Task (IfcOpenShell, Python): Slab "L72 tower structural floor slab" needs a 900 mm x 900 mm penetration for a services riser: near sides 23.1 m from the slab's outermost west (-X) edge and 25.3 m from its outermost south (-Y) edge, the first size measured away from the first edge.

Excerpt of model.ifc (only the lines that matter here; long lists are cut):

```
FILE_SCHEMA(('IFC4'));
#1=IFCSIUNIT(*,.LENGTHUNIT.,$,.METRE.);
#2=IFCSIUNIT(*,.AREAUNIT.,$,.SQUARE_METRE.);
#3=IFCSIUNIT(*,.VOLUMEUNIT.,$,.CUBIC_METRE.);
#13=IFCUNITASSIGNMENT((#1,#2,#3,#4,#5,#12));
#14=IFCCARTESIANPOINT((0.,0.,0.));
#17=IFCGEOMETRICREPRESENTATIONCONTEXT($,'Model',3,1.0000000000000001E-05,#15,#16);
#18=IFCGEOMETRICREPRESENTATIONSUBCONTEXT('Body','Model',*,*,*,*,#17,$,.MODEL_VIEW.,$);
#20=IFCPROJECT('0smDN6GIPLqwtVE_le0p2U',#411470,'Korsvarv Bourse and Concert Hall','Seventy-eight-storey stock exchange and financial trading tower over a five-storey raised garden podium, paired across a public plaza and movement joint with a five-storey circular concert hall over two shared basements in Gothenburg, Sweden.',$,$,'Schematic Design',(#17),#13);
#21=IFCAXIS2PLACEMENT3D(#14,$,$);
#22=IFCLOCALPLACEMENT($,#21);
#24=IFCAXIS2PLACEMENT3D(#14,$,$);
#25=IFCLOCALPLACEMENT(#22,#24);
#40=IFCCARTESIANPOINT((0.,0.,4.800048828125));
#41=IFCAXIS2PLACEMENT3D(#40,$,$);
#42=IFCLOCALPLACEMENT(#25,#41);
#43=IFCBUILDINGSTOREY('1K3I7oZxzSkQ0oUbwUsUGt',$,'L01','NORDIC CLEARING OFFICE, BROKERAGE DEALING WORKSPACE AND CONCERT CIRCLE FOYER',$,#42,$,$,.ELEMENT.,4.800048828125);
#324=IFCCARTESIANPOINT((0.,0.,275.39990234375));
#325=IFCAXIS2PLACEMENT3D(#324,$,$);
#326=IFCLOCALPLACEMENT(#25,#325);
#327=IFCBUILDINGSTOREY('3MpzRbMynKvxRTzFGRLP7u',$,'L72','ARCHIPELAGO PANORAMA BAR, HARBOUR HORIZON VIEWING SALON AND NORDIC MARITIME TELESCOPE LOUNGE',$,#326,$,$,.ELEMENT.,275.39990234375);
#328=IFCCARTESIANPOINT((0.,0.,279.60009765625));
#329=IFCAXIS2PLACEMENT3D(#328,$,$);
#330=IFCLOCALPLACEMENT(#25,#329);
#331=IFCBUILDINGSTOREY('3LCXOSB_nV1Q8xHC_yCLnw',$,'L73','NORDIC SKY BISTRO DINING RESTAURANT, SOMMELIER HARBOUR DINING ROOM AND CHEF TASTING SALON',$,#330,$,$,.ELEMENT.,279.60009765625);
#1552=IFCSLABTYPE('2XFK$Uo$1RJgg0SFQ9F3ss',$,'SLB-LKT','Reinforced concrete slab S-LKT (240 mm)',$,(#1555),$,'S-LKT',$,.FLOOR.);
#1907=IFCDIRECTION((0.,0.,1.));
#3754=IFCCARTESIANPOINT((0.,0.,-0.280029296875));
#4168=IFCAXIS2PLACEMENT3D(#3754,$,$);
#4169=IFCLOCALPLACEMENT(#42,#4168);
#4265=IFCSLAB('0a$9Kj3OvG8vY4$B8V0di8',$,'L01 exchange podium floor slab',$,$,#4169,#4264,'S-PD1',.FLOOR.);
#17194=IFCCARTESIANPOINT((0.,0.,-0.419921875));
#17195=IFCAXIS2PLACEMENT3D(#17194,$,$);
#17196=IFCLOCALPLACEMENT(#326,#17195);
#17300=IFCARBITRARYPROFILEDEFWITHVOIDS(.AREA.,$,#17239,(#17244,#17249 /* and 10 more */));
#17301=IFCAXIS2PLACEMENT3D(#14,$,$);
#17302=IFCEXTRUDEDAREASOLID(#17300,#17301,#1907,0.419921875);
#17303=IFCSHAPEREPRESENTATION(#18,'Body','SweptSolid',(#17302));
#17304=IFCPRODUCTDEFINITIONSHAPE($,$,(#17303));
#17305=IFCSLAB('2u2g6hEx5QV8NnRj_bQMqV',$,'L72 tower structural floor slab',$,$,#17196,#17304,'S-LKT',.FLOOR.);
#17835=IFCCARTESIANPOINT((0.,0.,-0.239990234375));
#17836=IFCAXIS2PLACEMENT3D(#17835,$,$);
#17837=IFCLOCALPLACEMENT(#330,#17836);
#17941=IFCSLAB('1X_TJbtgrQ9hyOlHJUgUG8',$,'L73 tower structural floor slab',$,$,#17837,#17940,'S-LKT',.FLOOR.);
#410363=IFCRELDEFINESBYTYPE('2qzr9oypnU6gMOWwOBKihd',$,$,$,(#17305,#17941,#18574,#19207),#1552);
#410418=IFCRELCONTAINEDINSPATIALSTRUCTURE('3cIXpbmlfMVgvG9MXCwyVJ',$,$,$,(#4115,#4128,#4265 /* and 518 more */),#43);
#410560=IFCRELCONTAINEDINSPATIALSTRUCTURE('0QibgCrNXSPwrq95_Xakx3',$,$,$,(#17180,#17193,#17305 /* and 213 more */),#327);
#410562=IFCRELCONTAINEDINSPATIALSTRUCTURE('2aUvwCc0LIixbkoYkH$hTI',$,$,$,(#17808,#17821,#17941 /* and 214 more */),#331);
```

```python
import numpy as np
import ifcopenshell
import ifcopenshell.api.feature
import ifcopenshell.api.geometry
import ifcopenshell.api.root
import ifcopenshell.geom
import ifcopenshell.util.placement
import ifcopenshell.util.representation
import ifcopenshell.util.shape
import ifcopenshell.util.unit

model = ifcopenshell.open("model.ifc")
unit_scale = ifcopenshell.util.unit.calculate_unit_scale(model)
settings = ifcopenshell.geom.settings()


def volume(element):
    """Net volume in cubic metres, openings subtracted."""
    shape = ifcopenshell.geom.create_shape(settings, element)
    return ifcopenshell.util.shape.get_volume(shape.geometry)


slab = model.by_guid("2u2g6hEx5QV8NnRj_bQMqV")
before = volume(slab)

# Extent in the slab's own axes, in metres. The edges named are its -X and -Y sides.
slab_shape = ifcopenshell.geom.create_shape(settings, slab)
vertices = ifcopenshell.util.shape.get_vertices(slab_shape.geometry)
x_min, y_min, bottom = vertices.min(axis=0)
top = vertices[:, 2].max()

opening = ifcopenshell.api.root.create_entity(model, ifc_class="IfcOpeningElement", name="Services riser opening", predefined_type="OPENING")
context = ifcopenshell.util.representation.get_context(model, "Model", "Body", "MODEL_VIEW")
width, depth = 0.9, 0.9
outline = [(0.0, 0.0), (width, 0.0), (width, depth), (0.0, depth), (0.0, 0.0)]
# Overshoot both faces by 50 mm so the cut is clean.
shape = ifcopenshell.api.geometry.add_slab_representation(
    model, context=context, depth=top - bottom + 0.1, polyline=outline
)
ifcopenshell.api.geometry.assign_representation(model, product=opening, representation=shape)

matrix = ifcopenshell.util.placement.get_local_placement(slab.ObjectPlacement)
matrix[:, 3] = matrix @ np.append(np.array([x_min + 23.1, y_min + 25.3, bottom - 0.05]) / unit_scale, 1.0)
ifcopenshell.api.geometry.edit_object_placement(model, product=opening, matrix=matrix, is_si=False)
ifcopenshell.api.feature.add_feature(model, feature=opening, element=slab)

after = volume(slab)

print(f"slab volume {before:.3f} -> {after:.3f} m3")

model.write("model_rev.ifc")
```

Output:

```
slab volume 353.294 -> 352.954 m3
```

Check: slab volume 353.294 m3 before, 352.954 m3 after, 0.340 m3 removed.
